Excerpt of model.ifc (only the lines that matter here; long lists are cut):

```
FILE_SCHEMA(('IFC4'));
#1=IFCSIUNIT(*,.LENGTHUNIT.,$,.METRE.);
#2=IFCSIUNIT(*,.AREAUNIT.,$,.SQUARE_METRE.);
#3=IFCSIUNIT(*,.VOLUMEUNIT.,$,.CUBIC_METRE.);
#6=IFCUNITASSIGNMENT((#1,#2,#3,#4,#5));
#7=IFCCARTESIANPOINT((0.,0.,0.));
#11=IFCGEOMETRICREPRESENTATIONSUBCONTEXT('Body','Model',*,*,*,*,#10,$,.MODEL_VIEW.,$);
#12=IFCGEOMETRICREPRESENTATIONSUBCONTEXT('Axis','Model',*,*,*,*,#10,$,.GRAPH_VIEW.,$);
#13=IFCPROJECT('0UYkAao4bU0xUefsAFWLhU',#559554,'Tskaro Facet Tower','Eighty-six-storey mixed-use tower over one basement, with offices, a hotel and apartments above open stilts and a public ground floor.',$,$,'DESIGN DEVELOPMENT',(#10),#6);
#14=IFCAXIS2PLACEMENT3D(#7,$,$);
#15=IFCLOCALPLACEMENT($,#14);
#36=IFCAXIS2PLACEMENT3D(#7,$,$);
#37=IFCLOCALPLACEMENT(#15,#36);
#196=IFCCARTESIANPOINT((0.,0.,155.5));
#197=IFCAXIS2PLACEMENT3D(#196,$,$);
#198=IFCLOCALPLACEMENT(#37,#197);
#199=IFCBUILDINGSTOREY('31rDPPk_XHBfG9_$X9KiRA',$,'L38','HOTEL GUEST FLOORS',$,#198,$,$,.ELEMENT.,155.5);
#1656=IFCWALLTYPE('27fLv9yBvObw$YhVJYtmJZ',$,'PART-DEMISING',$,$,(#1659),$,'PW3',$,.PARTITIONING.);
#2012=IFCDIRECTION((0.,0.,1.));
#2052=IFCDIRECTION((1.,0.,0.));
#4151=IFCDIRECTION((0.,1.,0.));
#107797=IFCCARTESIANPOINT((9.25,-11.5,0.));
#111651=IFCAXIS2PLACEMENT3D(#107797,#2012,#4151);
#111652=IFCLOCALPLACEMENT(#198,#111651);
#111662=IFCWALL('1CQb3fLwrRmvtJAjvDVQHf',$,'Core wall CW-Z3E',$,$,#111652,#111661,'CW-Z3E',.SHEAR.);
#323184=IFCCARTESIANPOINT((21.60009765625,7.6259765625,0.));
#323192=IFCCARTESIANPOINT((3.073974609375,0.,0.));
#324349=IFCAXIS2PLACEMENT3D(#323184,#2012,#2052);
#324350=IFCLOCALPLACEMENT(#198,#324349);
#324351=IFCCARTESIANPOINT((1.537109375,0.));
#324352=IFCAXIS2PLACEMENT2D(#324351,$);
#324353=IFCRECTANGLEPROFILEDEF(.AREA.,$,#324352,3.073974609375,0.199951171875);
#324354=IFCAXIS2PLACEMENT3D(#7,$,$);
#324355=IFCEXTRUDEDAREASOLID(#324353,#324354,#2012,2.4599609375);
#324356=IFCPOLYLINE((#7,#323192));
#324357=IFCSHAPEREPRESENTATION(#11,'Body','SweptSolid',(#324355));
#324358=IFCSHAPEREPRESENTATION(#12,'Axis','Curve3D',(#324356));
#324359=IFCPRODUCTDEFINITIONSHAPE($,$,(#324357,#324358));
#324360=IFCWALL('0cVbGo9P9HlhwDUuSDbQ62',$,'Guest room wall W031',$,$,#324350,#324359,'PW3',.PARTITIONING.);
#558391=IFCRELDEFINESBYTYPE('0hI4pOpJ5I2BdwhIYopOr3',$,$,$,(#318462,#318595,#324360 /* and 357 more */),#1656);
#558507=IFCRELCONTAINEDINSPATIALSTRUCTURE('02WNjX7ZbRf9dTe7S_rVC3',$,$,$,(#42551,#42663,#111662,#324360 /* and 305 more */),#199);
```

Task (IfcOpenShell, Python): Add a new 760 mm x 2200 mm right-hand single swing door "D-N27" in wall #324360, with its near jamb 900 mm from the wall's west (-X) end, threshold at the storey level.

```python
import numpy as np
import ifcopenshell
import ifcopenshell.api.feature
import ifcopenshell.api.geometry
import ifcopenshell.api.root
import ifcopenshell.api.spatial
import ifcopenshell.geom
import ifcopenshell.util.element
import ifcopenshell.util.placement
import ifcopenshell.util.representation
import ifcopenshell.util.shape
import ifcopenshell.util.unit

model = ifcopenshell.open("model.ifc")
unit_scale = ifcopenshell.util.unit.calculate_unit_scale(model)
settings = ifcopenshell.geom.settings()


def volume(element):
    """Net volume in cubic metres, openings subtracted."""
    shape = ifcopenshell.geom.create_shape(settings, element)
    return ifcopenshell.util.shape.get_volume(shape.geometry)


wall = model.by_guid("0cVbGo9P9HlhwDUuSDbQ62")
storey = ifcopenshell.util.element.get_container(wall, ifc_class="IfcBuildingStorey")
context = ifcopenshell.util.representation.get_context(model, "Model", "Body", "MODEL_VIEW")
before = volume(wall)

width, height, from_end, sill = 0.76, 2.2, 0.9, 0.0  # metres

# The wall runs along its own X axis, and the end named is its -X end.
wall_shape = ifcopenshell.geom.create_shape(settings, wall)
x, y, z = ifcopenshell.util.shape.get_vertices(wall_shape.geometry).T
start = x.min() + from_end
face, thickness = float(y.min()), float(y.max() - y.min())
wall_matrix = ifcopenshell.util.placement.get_local_placement(wall.ObjectPlacement)
level = ifcopenshell.util.placement.get_local_placement(storey.ObjectPlacement)[2, 3]


def in_wall(x, y):
    """Placement at x, y metres in the wall's axes, at sill height."""
    matrix = wall_matrix.copy()
    matrix[:, 3] = wall_matrix @ np.array([x / unit_scale, y / unit_scale, 0.0, 1.0])
    matrix[2, 3] = level + sill / unit_scale
    return matrix


# Opening: a box that overshoots both wall faces by 50 mm.
opening = ifcopenshell.api.root.create_entity(model, ifc_class="IfcOpeningElement", predefined_type="OPENING")
box = ifcopenshell.api.geometry.add_wall_representation(
    model, context=context, length=width, height=height, thickness=thickness + 0.1
)
ifcopenshell.api.geometry.assign_representation(model, product=opening, representation=box)
ifcopenshell.api.geometry.edit_object_placement(model, product=opening, matrix=in_wall(start, face - 0.05), is_si=False)
ifcopenshell.api.feature.add_feature(model, feature=opening, element=wall)

door = ifcopenshell.api.root.create_entity(model, ifc_class="IfcDoor", name="D-N27", predefined_type="DOOR")
door.OverallWidth, door.OverallHeight = width / unit_scale, height / unit_scale
door.OperationType = "SINGLE_SWING_RIGHT"
body = ifcopenshell.api.geometry.add_door_representation(
    model,
    context=context,
    overall_width=door.OverallWidth,
    overall_height=door.OverallHeight,
    operation_type="SINGLE_SWING_RIGHT",
    lining_properties={"LiningDepth": thickness / unit_scale, "ThresholdDepth": thickness / unit_scale},
)
ifcopenshell.api.geometry.assign_representation(model, product=door, representation=body)
ifcopenshell.api.spatial.assign_container(model, products=[door], relating_structure=storey)
ifcopenshell.api.feature.add_filling(model, opening=opening, element=door)

# The lining spans the wall, so the door starts at the wall face.
ifcopenshell.api.geometry.edit_object_placement(model, product=door, matrix=in_wall(start, face), is_si=False)

after = volume(wall)

print(f"wall volume {before:.3f} -> {after:.3f} m3")

model.write("model_rev.ifc")
```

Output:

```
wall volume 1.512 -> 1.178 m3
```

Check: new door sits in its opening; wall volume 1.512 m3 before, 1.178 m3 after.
